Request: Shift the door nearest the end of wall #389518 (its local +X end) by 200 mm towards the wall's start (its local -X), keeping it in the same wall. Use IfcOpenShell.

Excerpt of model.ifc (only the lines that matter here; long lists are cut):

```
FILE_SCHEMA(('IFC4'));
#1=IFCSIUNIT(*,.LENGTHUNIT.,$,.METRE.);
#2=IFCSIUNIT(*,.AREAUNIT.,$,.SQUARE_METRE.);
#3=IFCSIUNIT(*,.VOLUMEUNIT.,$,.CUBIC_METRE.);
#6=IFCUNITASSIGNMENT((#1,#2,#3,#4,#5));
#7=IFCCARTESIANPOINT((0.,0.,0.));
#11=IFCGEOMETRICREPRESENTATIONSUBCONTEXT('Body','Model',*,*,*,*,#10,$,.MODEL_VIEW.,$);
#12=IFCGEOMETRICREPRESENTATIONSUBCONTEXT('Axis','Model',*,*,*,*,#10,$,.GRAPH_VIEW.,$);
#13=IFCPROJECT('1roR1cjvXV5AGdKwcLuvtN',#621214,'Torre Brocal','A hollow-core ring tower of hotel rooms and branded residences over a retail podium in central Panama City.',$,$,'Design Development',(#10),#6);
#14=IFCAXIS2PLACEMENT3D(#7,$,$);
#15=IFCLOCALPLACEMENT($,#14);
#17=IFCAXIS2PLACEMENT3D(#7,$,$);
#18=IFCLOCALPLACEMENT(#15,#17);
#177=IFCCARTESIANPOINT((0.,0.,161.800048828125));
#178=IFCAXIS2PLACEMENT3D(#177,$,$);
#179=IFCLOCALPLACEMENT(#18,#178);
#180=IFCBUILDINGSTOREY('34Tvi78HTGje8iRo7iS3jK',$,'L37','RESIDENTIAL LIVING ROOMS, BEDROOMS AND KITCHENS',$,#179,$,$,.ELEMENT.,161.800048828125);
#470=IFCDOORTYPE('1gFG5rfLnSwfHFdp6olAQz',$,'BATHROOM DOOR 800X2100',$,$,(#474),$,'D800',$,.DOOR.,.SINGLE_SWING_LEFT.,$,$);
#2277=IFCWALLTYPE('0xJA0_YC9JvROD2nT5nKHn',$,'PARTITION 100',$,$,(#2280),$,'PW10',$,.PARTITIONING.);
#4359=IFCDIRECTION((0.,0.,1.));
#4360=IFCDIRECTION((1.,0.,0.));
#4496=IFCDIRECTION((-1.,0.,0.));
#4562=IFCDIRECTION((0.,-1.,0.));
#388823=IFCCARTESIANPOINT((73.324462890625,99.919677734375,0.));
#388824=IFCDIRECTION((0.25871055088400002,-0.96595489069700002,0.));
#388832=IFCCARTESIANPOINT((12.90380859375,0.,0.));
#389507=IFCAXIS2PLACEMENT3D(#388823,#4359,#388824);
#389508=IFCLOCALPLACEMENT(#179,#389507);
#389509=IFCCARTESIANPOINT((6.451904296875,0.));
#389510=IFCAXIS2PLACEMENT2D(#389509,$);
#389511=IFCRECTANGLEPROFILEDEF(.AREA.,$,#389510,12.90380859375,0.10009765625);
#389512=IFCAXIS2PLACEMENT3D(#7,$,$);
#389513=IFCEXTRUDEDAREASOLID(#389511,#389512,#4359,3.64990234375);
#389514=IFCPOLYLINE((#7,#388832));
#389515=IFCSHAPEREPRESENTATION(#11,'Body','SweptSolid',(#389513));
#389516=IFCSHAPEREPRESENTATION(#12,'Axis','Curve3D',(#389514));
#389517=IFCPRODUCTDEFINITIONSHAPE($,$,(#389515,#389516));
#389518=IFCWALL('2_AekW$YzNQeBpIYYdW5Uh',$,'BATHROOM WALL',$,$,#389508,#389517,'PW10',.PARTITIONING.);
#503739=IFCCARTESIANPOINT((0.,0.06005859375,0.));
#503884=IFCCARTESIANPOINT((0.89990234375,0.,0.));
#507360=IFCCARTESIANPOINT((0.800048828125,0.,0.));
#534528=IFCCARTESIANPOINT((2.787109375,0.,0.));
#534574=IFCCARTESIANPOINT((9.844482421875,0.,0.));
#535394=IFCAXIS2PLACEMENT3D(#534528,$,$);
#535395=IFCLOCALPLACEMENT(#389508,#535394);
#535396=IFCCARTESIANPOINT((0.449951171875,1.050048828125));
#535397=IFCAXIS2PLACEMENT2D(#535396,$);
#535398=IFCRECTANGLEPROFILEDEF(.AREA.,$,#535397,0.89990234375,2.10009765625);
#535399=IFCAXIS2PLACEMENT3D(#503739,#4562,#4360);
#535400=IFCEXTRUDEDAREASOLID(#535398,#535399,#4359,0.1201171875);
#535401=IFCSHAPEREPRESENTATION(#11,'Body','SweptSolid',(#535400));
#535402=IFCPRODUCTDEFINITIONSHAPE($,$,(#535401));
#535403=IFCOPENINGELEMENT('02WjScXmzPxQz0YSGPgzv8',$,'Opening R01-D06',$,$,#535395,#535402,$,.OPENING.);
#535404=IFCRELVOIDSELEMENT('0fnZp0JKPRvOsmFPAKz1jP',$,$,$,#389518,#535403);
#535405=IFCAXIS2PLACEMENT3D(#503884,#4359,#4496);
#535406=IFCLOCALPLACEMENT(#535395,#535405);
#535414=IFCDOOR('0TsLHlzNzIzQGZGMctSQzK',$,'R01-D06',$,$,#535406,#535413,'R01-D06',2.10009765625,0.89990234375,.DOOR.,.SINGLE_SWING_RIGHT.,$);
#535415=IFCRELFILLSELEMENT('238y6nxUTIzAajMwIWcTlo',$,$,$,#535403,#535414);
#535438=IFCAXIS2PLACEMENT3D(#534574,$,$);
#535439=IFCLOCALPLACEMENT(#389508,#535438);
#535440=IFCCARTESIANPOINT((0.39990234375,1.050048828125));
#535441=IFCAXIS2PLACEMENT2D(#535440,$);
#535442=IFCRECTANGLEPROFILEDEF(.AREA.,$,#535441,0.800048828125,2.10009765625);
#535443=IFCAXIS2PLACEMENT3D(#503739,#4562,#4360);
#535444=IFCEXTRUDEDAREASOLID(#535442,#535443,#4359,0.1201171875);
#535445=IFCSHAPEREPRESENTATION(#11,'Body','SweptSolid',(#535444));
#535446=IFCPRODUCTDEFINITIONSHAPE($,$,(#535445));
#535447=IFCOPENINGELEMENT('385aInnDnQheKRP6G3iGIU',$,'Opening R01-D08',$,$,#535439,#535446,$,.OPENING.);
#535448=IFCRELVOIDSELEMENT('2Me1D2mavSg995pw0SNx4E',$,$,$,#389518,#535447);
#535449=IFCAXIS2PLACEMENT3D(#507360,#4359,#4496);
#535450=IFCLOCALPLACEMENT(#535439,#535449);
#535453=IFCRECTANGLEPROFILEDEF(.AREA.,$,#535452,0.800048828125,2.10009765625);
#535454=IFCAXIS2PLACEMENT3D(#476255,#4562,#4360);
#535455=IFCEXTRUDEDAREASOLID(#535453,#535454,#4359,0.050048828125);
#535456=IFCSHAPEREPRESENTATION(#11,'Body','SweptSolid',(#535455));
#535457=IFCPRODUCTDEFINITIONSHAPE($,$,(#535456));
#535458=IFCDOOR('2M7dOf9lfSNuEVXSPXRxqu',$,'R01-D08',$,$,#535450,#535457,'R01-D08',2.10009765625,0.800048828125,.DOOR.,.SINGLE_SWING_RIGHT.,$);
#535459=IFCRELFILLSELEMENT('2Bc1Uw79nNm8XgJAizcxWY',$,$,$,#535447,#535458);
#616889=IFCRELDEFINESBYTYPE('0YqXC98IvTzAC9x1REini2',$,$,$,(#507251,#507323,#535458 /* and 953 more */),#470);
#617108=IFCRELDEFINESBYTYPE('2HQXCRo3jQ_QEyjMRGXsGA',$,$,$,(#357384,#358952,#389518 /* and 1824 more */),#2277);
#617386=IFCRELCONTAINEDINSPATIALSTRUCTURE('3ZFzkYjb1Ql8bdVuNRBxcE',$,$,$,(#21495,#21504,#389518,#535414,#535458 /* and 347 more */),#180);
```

```python
import ifcopenshell
import ifcopenshell.api.geometry
import ifcopenshell.util.placement
import ifcopenshell.util.unit

model = ifcopenshell.open("model.ifc")
unit_scale = ifcopenshell.util.unit.calculate_unit_scale(model)

door = model.by_guid("2M7dOf9lfSNuEVXSPXRxqu")
opening = door.FillsVoids[0].RelatingOpeningElement
wall = opening.VoidsElements[0].RelatingBuildingElement

wall_matrix = ifcopenshell.util.placement.get_local_placement(wall.ObjectPlacement)
shift = wall_matrix[:3, 0] * -0.2 / unit_scale
before = ifcopenshell.util.placement.get_local_placement(door.ObjectPlacement)[:3, 3].copy()

# The door is placed relative to its opening, so it follows when the opening moves.
matrix = ifcopenshell.util.placement.get_local_placement(opening.ObjectPlacement)
matrix[:3, 3] += shift
ifcopenshell.api.geometry.edit_object_placement(
    model, product=opening, matrix=matrix, is_si=False, should_transform_children=True
)

after = ifcopenshell.util.placement.get_local_placement(door.ObjectPlacement)[:3, 3]
print("door moved by", (after - before).round(3) + 0.0)

model.write("model_updated.ifc")
```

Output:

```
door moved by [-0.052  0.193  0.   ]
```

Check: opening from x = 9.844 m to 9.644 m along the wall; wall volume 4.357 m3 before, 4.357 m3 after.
